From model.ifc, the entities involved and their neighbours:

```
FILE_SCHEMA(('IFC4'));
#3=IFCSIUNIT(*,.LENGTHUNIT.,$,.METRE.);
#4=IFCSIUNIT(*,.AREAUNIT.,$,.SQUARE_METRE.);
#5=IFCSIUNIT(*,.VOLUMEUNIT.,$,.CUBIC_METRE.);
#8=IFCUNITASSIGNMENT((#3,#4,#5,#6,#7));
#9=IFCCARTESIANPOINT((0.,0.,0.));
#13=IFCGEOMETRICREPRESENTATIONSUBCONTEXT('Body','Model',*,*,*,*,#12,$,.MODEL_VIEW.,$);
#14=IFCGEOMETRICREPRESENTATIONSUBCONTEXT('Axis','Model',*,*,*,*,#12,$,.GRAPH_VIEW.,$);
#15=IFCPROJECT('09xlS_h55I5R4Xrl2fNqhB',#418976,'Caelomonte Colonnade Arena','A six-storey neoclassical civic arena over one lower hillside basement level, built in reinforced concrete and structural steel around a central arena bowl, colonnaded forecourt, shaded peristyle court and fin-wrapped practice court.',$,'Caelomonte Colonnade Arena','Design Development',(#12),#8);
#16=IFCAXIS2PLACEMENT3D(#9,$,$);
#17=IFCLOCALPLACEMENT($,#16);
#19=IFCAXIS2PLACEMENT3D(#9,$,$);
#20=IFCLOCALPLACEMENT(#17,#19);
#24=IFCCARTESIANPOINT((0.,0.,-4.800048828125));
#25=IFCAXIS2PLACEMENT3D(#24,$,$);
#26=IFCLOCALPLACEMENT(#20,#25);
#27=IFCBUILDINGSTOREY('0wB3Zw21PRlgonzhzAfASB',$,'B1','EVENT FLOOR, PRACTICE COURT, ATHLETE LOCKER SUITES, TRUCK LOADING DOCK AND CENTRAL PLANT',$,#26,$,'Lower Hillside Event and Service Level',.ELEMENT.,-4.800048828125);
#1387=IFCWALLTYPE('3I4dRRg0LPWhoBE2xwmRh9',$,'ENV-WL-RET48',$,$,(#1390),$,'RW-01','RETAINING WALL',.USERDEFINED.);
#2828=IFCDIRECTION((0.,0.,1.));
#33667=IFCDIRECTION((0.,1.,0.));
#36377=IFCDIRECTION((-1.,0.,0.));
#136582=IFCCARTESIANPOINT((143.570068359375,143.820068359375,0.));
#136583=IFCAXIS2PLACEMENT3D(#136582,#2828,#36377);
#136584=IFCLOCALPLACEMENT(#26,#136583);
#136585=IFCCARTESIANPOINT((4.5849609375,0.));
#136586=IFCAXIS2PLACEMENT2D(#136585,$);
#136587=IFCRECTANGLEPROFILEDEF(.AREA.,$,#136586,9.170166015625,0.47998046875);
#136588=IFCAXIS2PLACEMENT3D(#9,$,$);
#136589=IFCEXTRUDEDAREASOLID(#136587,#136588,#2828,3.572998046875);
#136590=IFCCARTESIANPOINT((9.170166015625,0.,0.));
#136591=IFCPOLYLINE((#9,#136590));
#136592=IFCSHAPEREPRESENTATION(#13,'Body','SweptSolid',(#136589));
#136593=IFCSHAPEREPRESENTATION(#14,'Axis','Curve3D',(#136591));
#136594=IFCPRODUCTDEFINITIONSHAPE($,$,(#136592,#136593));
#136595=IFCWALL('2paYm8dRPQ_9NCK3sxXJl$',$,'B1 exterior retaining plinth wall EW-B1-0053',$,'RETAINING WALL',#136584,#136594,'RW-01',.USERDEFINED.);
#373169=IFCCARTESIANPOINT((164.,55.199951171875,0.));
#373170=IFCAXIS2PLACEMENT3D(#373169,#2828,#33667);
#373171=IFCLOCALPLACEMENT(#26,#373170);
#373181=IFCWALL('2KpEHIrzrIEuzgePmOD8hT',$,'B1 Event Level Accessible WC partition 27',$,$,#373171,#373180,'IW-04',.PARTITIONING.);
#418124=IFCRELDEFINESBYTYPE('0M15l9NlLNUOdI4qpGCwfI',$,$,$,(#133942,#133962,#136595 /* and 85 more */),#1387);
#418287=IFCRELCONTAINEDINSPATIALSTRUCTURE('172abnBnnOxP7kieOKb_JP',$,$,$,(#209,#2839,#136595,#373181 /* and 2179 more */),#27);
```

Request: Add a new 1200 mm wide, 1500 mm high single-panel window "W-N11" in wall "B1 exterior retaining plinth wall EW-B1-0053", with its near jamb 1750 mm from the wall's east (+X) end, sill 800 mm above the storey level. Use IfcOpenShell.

```python
import numpy as np
import ifcopenshell
import ifcopenshell.api.feature
import ifcopenshell.api.geometry
import ifcopenshell.api.root
import ifcopenshell.api.spatial
import ifcopenshell.geom
import ifcopenshell.util.element
import ifcopenshell.util.placement
import ifcopenshell.util.representation
import ifcopenshell.util.shape
import ifcopenshell.util.unit

model = ifcopenshell.open("model.ifc")
unit_scale = ifcopenshell.util.unit.calculate_unit_scale(model)
settings = ifcopenshell.geom.settings()


def volume(element):
    """Net volume in cubic metres, openings subtracted."""
    shape = ifcopenshell.geom.create_shape(settings, element)
    return ifcopenshell.util.shape.get_volume(shape.geometry)


wall = model.by_guid("2paYm8dRPQ_9NCK3sxXJl$")
storey = ifcopenshell.util.element.get_container(wall, ifc_class="IfcBuildingStorey")
context = ifcopenshell.util.representation.get_context(model, "Model", "Body", "MODEL_VIEW")
before = volume(wall)

width, height, from_end, sill = 1.2, 1.5, 1.75, 0.8  # metres

# The wall runs along its own X axis, and the end named is its -X end.
wall_shape = ifcopenshell.geom.create_shape(settings, wall)
x, y, z = ifcopenshell.util.shape.get_vertices(wall_shape.geometry).T
start = x.min() + from_end
face, thickness = float(y.min()), float(y.max() - y.min())
wall_matrix = ifcopenshell.util.placement.get_local_placement(wall.ObjectPlacement)
level = ifcopenshell.util.placement.get_local_placement(storey.ObjectPlacement)[2, 3]


def in_wall(x, y):
    """Placement at x, y metres in the wall's axes, at sill height."""
    matrix = wall_matrix.copy()
    matrix[:, 3] = wall_matrix @ np.array([x / unit_scale, y / unit_scale, 0.0, 1.0])
    matrix[2, 3] = level + sill / unit_scale
    return matrix


# Opening: a box that overshoots both wall faces by 50 mm.
opening = ifcopenshell.api.root.create_entity(model, ifc_class="IfcOpeningElement", predefined_type="OPENING")
box = ifcopenshell.api.geometry.add_wall_representation(
    model, context=context, length=width, height=height, thickness=thickness + 0.1
)
ifcopenshell.api.geometry.assign_representation(model, product=opening, representation=box)
ifcopenshell.api.geometry.edit_object_placement(model, product=opening, matrix=in_wall(start, face - 0.05), is_si=False)
ifcopenshell.api.feature.add_feature(model, feature=opening, element=wall)

window = ifcopenshell.api.root.create_entity(model, ifc_class="IfcWindow", name="W-N11", predefined_type="WINDOW")
window.OverallWidth, window.OverallHeight = width / unit_scale, height / unit_scale
window.PartitioningType = "SINGLE_PANEL"
body = ifcopenshell.api.geometry.add_window_representation(
    model,
    context=context,
    overall_width=window.OverallWidth,
    overall_height=window.OverallHeight,
    partition_type="SINGLE_PANEL",
)
ifcopenshell.api.geometry.assign_representation(model, product=window, representation=body)
ifcopenshell.api.spatial.assign_container(model, products=[window], relating_structure=storey)
ifcopenshell.api.feature.add_filling(model, opening=opening, element=window)

# Centre the window in the wall's thickness.
ifcopenshell.api.geometry.edit_object_placement(model, product=window, matrix=in_wall(start, face), is_si=False)
window_shape = ifcopenshell.geom.create_shape(settings, window)
depth = ifcopenshell.util.shape.get_vertices(window_shape.geometry)[:, 1]
offset = face + thickness / 2 - (depth.min() + depth.max()) / 2
ifcopenshell.api.geometry.edit_object_placement(model, product=window, matrix=in_wall(start, offset), is_si=False)

after = volume(wall)

print(f"wall volume {before:.3f} -> {after:.3f} m3")

model.write("model_rev.ifc")
```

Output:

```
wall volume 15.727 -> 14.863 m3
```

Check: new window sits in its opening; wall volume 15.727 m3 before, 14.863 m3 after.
